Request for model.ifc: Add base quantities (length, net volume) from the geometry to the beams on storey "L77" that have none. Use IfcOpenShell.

First a look at what the model holds.

```python
import ifcopenshell
import ifcopenshell.util.element
import ifcopenshell.util.unit

model = ifcopenshell.open("model.ifc")
print(model.schema)
for unit_type in ("LENGTHUNIT", "AREAUNIT", "VOLUMEUNIT"):
    print(unit_type, ifcopenshell.util.unit.calculate_unit_scale(model, unit_type))
storey = next(s for s in model.by_type("IfcBuildingStorey") if s.Name == "L77")
beams = [e for e in ifcopenshell.util.element.get_decomposition(storey) if e.is_a("IfcBeam")]
for e in sorted(beams, key=lambda e: e.id()):
    print(e.id(), e.is_a(), e.Name, list(ifcopenshell.util.element.get_psets(e, qtos_only=True)), sep=" | ")
```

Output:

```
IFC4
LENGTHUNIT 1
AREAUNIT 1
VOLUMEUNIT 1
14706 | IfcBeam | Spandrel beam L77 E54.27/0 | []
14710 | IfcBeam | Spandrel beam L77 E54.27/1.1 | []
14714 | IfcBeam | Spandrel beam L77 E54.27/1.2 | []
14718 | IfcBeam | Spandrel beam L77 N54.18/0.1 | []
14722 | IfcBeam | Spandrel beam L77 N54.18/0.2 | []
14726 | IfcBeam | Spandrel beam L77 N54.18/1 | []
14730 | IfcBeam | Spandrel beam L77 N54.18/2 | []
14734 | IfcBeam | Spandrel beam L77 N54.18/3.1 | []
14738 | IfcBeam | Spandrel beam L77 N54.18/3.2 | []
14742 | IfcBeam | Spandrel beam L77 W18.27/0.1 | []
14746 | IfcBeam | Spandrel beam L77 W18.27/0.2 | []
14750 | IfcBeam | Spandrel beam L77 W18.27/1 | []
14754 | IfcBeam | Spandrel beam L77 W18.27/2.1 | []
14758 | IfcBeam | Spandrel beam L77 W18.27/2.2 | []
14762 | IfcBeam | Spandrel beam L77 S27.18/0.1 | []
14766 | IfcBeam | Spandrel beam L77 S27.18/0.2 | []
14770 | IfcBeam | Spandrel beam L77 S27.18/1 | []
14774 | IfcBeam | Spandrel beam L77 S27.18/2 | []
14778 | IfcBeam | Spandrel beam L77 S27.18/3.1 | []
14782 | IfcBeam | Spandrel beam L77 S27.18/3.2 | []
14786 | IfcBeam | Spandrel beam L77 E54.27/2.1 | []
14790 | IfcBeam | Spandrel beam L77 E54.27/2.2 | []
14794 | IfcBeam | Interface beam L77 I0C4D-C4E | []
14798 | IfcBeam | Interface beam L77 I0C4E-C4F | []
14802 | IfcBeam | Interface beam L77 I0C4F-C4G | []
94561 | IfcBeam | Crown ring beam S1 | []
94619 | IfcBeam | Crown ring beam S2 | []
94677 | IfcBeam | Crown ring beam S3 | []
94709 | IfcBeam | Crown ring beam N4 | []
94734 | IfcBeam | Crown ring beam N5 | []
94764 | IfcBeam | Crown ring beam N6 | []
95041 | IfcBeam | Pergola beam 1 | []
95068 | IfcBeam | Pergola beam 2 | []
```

```python
import ifcopenshell
import ifcopenshell.api.pset
import ifcopenshell.geom
import ifcopenshell.util.element
import ifcopenshell.util.shape
import ifcopenshell.util.unit

model = ifcopenshell.open("model.ifc")
unit_scale = ifcopenshell.util.unit.calculate_unit_scale(model)
volume_scale = ifcopenshell.util.unit.calculate_unit_scale(model, "VOLUMEUNIT")
settings = ifcopenshell.geom.settings()

storey = next(s for s in model.by_type("IfcBuildingStorey") if s.Name == "L77")
beams = [e for e in ifcopenshell.util.element.get_decomposition(storey) if e.is_a("IfcBeam")]

for e in sorted(beams, key=lambda e: e.id()):
    if ifcopenshell.util.element.get_psets(e, qtos_only=True, should_inherit=False):
        continue
    # Geometry comes back in metres, in the element's own axes.
    shape = ifcopenshell.geom.create_shape(settings, e)
    values = {
        "Length": ifcopenshell.util.shape.get_max_xyz(shape.geometry) / unit_scale,
        "NetVolume": ifcopenshell.util.shape.get_volume(shape.geometry) / volume_scale,
    }
    qto = ifcopenshell.api.pset.add_qto(model, product=e, name="Qto_BeamBaseQuantities")
    ifcopenshell.api.pset.edit_qto(model, qto=qto, properties=values)
    print(e.id(), {k: round(v, 3) for k, v in values.items()})

model.write("model_updated.ifc")
```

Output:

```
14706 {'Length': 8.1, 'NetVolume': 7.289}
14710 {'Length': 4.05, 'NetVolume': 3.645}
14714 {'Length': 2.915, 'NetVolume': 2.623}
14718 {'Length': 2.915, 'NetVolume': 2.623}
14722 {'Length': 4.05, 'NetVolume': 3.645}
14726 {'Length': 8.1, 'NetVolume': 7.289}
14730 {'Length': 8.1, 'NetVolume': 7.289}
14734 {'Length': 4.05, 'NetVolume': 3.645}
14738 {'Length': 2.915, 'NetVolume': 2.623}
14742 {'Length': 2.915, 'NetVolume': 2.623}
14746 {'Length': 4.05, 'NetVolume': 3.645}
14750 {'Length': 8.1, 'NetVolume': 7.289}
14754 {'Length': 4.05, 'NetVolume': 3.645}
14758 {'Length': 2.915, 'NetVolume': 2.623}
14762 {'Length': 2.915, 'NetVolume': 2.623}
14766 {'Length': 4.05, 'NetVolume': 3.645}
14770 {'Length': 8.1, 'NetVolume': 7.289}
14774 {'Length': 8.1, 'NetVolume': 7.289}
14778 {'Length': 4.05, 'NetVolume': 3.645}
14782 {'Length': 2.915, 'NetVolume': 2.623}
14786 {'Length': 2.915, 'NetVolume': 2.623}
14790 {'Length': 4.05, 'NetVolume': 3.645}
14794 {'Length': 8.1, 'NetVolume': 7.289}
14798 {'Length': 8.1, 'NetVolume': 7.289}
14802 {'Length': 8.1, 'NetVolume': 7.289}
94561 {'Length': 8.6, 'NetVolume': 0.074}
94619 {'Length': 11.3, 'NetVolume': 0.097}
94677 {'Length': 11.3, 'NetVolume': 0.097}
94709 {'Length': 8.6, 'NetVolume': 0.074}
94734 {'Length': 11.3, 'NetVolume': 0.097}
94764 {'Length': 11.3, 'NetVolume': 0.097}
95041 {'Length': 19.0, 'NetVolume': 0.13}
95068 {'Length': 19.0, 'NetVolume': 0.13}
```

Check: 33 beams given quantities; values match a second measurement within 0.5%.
